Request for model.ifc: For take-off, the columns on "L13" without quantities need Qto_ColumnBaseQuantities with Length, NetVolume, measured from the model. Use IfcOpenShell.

First a look at what the model holds.

```python
import ifcopenshell
import ifcopenshell.util.element
import ifcopenshell.util.unit

model = ifcopenshell.open("model.ifc")
print(model.schema)
for unit_type in ("LENGTHUNIT", "AREAUNIT", "VOLUMEUNIT"):
    print(unit_type, ifcopenshell.util.unit.calculate_unit_scale(model, unit_type))
storey = next(s for s in model.by_type("IfcBuildingStorey") if s.Name == "L13")
columns = [e for e in ifcopenshell.util.element.get_decomposition(storey) if e.is_a("IfcColumn")]
for e in sorted(columns, key=lambda e: e.id()):
    print(e.id(), e.is_a(), e.Name, list(ifcopenshell.util.element.get_psets(e, qtos_only=True)), sep=" | ")
```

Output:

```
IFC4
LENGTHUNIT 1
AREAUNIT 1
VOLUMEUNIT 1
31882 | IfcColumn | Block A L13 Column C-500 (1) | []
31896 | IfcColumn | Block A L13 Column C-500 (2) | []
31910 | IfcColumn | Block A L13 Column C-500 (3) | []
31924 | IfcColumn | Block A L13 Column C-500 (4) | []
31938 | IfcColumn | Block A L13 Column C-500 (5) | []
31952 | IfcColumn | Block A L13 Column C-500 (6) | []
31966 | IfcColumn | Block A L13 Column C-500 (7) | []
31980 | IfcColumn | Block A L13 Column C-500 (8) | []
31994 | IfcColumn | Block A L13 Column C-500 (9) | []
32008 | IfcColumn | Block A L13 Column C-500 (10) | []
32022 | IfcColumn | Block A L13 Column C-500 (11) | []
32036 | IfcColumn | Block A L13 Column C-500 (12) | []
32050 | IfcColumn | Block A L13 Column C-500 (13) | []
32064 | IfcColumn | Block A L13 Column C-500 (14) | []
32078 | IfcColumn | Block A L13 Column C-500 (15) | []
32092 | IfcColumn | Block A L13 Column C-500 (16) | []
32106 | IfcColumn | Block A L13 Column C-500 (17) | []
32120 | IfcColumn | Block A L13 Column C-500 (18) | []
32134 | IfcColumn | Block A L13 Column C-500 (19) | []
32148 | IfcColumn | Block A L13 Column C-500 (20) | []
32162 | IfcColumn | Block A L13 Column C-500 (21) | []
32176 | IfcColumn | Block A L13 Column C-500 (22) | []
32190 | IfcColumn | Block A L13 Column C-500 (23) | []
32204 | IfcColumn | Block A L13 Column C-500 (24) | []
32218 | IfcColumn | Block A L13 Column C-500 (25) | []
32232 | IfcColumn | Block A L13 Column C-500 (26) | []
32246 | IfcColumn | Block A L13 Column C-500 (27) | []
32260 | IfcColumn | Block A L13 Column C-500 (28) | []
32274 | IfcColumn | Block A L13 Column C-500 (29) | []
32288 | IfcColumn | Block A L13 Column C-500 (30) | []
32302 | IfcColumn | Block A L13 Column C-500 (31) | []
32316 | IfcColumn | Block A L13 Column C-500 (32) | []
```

```python
import ifcopenshell
import ifcopenshell.api.pset
import ifcopenshell.geom
import ifcopenshell.util.element
import ifcopenshell.util.shape
import ifcopenshell.util.unit

model = ifcopenshell.open("model.ifc")
unit_scale = ifcopenshell.util.unit.calculate_unit_scale(model)
volume_scale = ifcopenshell.util.unit.calculate_unit_scale(model, "VOLUMEUNIT")
settings = ifcopenshell.geom.settings()

storey = next(s for s in model.by_type("IfcBuildingStorey") if s.Name == "L13")
columns = [e for e in ifcopenshell.util.element.get_decomposition(storey) if e.is_a("IfcColumn")]

for e in sorted(columns, key=lambda e: e.id()):
    if ifcopenshell.util.element.get_psets(e, qtos_only=True, should_inherit=False):
        continue
    # Geometry comes back in metres, in the element's own axes.
    shape = ifcopenshell.geom.create_shape(settings, e)
    values = {
        "Length": ifcopenshell.util.shape.get_z(shape.geometry) / unit_scale,
        "NetVolume": ifcopenshell.util.shape.get_volume(shape.geometry) / volume_scale,
    }
    qto = ifcopenshell.api.pset.add_qto(model, product=e, name="Qto_ColumnBaseQuantities")
    ifcopenshell.api.pset.edit_qto(model, qto=qto, properties=values)
    print(e.id(), {k: round(v, 3) for k, v in values.items()})

model.write("model_rev.ifc")
```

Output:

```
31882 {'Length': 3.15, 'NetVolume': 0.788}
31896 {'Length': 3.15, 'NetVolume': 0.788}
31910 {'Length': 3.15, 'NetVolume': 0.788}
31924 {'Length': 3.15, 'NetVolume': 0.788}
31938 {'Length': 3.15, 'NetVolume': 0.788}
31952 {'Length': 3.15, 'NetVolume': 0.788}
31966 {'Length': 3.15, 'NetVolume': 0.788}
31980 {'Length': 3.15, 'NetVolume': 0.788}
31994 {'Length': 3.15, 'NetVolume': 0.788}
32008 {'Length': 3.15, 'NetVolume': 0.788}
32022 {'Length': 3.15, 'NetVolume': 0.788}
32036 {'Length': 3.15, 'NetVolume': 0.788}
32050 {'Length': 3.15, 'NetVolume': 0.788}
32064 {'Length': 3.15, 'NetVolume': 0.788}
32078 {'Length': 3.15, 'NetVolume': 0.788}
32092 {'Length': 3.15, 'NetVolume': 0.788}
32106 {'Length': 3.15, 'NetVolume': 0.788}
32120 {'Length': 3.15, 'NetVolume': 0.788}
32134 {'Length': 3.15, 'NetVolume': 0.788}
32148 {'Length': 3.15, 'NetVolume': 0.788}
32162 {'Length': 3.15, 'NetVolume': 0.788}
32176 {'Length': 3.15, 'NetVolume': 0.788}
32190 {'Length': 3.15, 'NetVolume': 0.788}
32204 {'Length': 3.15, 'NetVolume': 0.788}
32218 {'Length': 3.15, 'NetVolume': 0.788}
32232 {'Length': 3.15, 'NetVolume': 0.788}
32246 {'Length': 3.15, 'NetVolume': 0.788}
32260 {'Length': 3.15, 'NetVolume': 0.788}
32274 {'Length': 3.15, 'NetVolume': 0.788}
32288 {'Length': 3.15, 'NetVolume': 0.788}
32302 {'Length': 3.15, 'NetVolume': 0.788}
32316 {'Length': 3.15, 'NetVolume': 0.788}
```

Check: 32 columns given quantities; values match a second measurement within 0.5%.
